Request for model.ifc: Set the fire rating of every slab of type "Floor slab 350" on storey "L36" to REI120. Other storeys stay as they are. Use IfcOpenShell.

First a look at what the model holds.

```python
import ifcopenshell
import ifcopenshell.util.element

model = ifcopenshell.open("model.ifc")
print(model.schema)
storey = next(s for s in model.by_type("IfcBuildingStorey") if s.Name == "L36")
slabs = [e for e in ifcopenshell.util.element.get_decomposition(storey) if e.is_a("IfcSlab")]
seen = {}
for e in slabs:
    element_type = ifcopenshell.util.element.get_type(e)
    key = (element_type.Name if element_type != e and element_type else None, ifcopenshell.util.element.get_pset(e, "Pset_SlabCommon", "FireRating"))
    seen[key] = seen.get(key, 0) + 1
for (name, value), count in sorted(seen.items(), key=str):
    print(count, "x", name, "|", value)
```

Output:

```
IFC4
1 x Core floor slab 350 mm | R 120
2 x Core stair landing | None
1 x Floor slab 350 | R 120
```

```python
import ifcopenshell
import ifcopenshell.api.pset
import ifcopenshell.util.element

model = ifcopenshell.open("model.ifc")

storey = next(s for s in model.by_type("IfcBuildingStorey") if s.Name == "L36")
slabs = [e for e in ifcopenshell.util.element.get_decomposition(storey) if e.is_a("IfcSlab")]

count = 0
for e in slabs:
    element_type = ifcopenshell.util.element.get_type(e)
    if element_type in (None, e) or element_type.Name != "Floor slab 350":
        continue
    found = ifcopenshell.util.element.get_pset(e, "Pset_SlabCommon", should_inherit=False)
    if found:
        pset = model.by_id(found["id"])
        if len(ifcopenshell.util.element.get_elements_by_pset(pset)) > 1:
            pset = ifcopenshell.api.pset.unshare_pset(model, products=[e], pset=pset)[0]
    else:
        pset = ifcopenshell.api.pset.add_pset(model, product=e, name="Pset_SlabCommon")
    ifcopenshell.api.pset.edit_pset(model, pset=pset, properties={"FireRating": "REI120"})
    count += 1

print(count, "slabs updated")

model.write("model_edited.ifc")
```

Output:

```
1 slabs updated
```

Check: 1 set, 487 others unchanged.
